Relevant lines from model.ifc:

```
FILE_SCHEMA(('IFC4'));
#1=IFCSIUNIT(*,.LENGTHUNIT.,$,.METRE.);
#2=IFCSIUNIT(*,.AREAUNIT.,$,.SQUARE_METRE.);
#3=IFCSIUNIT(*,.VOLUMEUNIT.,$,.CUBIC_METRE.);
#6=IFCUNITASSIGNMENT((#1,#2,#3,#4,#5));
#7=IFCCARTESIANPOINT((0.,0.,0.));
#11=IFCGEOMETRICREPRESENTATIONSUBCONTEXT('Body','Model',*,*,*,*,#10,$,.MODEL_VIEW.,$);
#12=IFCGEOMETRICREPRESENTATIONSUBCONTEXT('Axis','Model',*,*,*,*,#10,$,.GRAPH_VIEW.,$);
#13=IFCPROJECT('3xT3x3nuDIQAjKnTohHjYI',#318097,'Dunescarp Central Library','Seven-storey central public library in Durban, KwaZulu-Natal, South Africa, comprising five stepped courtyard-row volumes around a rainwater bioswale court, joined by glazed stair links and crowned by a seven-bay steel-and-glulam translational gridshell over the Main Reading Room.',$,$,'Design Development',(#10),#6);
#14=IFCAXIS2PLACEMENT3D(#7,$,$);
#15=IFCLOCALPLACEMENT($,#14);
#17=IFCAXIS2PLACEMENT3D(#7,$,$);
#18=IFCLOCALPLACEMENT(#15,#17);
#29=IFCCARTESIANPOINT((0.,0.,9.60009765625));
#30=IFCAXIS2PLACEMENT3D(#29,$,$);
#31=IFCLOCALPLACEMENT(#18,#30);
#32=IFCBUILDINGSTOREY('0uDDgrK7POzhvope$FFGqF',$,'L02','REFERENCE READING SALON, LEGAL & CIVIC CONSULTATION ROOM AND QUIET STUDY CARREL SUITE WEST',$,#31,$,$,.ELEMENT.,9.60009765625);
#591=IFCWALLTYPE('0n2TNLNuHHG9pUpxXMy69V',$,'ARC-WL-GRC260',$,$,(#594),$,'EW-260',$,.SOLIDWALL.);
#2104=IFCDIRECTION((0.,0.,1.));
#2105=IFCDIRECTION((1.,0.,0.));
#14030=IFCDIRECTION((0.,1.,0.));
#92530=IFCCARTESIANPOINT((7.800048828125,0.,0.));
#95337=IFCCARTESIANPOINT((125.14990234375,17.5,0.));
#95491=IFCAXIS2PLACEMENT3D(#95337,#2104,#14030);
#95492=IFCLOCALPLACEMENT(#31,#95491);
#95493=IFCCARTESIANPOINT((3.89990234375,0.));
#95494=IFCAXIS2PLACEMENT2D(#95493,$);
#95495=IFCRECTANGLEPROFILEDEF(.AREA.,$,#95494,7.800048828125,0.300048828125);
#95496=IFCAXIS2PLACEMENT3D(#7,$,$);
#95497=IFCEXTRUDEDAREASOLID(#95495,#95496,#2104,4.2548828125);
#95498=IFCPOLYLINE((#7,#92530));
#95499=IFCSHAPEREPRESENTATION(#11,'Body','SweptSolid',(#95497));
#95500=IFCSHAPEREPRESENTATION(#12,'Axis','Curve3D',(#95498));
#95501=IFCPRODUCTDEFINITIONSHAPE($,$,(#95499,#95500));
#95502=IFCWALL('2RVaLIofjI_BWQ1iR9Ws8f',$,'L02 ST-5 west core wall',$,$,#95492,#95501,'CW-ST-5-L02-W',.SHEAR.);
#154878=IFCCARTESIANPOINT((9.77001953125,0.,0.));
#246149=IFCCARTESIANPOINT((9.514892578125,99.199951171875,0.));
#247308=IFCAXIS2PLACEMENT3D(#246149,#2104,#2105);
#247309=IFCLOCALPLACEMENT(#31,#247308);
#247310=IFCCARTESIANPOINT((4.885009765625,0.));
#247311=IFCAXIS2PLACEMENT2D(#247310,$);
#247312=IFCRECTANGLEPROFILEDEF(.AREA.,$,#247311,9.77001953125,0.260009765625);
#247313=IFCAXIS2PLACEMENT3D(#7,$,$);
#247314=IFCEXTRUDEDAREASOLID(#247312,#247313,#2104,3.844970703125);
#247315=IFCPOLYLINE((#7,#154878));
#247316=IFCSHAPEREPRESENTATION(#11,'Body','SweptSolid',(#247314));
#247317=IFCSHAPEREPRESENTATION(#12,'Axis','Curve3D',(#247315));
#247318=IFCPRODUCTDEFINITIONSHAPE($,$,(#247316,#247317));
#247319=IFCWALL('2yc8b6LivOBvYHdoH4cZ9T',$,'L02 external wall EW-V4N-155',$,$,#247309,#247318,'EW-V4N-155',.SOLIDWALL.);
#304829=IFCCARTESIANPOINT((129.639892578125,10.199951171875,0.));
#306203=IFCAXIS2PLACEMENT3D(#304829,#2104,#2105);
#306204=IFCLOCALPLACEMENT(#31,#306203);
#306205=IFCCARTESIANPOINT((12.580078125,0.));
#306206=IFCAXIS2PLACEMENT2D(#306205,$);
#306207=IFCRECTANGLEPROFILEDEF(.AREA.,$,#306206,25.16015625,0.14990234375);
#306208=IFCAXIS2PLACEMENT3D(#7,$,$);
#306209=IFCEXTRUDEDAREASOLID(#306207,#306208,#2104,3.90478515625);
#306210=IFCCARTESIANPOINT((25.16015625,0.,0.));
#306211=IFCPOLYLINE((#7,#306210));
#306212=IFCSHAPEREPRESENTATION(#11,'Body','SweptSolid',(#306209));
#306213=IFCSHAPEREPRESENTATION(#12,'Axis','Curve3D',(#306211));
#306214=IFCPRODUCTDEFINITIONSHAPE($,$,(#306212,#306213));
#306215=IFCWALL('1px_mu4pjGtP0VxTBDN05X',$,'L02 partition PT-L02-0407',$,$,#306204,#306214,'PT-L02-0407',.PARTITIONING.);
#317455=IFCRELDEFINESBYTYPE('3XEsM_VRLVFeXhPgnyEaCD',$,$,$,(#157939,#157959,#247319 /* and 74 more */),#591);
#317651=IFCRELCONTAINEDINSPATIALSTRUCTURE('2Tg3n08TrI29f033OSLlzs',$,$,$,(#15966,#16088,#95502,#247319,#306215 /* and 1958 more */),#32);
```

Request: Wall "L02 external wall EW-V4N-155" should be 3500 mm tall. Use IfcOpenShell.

```python
import ifcopenshell
import ifcopenshell.geom
import ifcopenshell.util.representation
import ifcopenshell.util.shape

model = ifcopenshell.open("model.ifc")
settings = ifcopenshell.geom.settings()


def volume(element):
    """Net volume in cubic metres, openings subtracted."""
    shape = ifcopenshell.geom.create_shape(settings, element)
    return ifcopenshell.util.shape.get_volume(shape.geometry)


wall = model.by_id(247319)
before = volume(wall)

body = ifcopenshell.util.representation.get_representation(wall, "Model", "Body")
solid = body.Items[0]
old_height = solid.Depth
solid.Depth = 3.5
after = volume(wall)

print(f"height {old_height:g} -> {solid.Depth:g}, volume {before:.3f} -> {after:.3f} m3")

model.write("model_v2.ifc")
```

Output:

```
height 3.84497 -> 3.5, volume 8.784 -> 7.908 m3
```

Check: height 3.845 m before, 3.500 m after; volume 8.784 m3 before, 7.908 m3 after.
